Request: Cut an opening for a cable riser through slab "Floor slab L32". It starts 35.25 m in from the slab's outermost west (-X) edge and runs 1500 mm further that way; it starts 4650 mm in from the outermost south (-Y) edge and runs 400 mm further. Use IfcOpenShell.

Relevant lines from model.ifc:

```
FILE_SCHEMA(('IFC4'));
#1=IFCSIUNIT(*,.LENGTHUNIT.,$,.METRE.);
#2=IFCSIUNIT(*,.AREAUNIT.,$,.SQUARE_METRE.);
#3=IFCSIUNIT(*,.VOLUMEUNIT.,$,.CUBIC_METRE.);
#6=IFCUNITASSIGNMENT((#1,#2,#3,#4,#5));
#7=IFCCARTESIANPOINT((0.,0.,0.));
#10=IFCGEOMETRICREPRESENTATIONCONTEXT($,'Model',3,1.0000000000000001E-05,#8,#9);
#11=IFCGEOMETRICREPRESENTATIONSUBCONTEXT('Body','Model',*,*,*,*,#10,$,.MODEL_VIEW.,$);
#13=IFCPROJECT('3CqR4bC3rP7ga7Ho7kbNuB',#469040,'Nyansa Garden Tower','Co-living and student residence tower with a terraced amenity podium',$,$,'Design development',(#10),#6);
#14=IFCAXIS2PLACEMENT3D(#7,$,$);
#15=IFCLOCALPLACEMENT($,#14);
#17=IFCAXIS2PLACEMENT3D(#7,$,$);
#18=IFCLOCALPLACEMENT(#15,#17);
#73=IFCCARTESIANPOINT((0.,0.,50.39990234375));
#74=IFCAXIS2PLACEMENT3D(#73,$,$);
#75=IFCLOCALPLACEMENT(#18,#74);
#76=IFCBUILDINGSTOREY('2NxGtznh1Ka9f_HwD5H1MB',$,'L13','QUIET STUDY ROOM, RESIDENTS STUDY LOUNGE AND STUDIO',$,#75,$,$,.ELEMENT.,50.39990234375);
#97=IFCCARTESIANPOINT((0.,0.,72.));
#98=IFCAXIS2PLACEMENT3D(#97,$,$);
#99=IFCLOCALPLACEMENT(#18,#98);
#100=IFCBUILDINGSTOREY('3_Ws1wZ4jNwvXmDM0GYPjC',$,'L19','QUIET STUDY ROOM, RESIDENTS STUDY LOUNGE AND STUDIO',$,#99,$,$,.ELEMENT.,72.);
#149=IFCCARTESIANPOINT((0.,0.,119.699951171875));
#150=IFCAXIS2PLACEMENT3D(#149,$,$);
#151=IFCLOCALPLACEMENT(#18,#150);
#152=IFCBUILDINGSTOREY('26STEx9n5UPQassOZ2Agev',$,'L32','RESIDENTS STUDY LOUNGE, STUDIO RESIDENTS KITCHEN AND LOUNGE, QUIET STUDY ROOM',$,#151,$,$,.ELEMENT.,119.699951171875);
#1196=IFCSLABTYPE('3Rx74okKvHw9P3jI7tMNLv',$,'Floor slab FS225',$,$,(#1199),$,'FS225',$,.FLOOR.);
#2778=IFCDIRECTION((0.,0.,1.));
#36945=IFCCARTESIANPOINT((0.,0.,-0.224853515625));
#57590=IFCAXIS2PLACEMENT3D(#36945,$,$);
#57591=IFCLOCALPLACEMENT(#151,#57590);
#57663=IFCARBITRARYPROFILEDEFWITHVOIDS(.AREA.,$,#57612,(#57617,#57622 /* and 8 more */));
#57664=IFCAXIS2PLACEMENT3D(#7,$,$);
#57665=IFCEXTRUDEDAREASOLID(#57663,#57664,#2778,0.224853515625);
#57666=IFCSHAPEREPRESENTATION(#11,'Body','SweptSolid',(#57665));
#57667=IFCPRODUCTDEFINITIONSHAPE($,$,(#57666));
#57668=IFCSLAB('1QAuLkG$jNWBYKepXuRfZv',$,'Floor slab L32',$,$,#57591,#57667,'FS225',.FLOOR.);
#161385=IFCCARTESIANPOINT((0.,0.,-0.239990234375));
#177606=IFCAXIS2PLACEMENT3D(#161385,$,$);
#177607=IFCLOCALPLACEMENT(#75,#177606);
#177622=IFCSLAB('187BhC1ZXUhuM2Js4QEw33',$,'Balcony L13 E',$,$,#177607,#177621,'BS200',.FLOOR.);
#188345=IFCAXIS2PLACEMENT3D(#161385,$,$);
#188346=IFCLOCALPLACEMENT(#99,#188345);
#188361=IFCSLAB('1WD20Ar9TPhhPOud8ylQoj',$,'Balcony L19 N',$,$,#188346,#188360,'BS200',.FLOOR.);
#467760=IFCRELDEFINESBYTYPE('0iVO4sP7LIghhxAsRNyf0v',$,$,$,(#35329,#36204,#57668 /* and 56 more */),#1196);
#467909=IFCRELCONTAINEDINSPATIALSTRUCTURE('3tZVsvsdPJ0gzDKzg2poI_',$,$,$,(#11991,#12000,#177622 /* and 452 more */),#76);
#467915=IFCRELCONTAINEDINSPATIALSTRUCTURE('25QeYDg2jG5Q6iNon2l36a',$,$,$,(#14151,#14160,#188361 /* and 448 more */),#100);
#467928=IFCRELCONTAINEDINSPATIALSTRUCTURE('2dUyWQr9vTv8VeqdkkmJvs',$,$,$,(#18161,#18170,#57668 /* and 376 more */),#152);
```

```python
import numpy as np
import ifcopenshell
import ifcopenshell.api.feature
import ifcopenshell.api.geometry
import ifcopenshell.api.root
import ifcopenshell.geom
import ifcopenshell.util.placement
import ifcopenshell.util.representation
import ifcopenshell.util.shape
import ifcopenshell.util.unit

model = ifcopenshell.open("model.ifc")
unit_scale = ifcopenshell.util.unit.calculate_unit_scale(model)
settings = ifcopenshell.geom.settings()


def volume(element):
    """Net volume in cubic metres, openings subtracted."""
    shape = ifcopenshell.geom.create_shape(settings, element)
    return ifcopenshell.util.shape.get_volume(shape.geometry)


slab = model.by_id(57668)
before = volume(slab)

# Extent in the slab's own axes, in metres. The edges named are its -X and -Y sides.
slab_shape = ifcopenshell.geom.create_shape(settings, slab)
vertices = ifcopenshell.util.shape.get_vertices(slab_shape.geometry)
x_min, y_min, bottom = vertices.min(axis=0)
top = vertices[:, 2].max()

opening = ifcopenshell.api.root.create_entity(model, ifc_class="IfcOpeningElement", name="Cable riser opening", predefined_type="OPENING")
context = ifcopenshell.util.representation.get_context(model, "Model", "Body", "MODEL_VIEW")
width, depth = 1.5, 0.4
outline = [(0.0, 0.0), (width, 0.0), (width, depth), (0.0, depth), (0.0, 0.0)]
# Overshoot both faces by 50 mm so the cut is clean.
shape = ifcopenshell.api.geometry.add_slab_representation(
    model, context=context, depth=top - bottom + 0.1, polyline=outline
)
ifcopenshell.api.geometry.assign_representation(model, product=opening, representation=shape)

matrix = ifcopenshell.util.placement.get_local_placement(slab.ObjectPlacement)
matrix[:, 3] = matrix @ np.append(np.array([x_min + 35.25, y_min + 4.65, bottom - 0.05]) / unit_scale, 1.0)
ifcopenshell.api.geometry.edit_object_placement(model, product=opening, matrix=matrix, is_si=False)
ifcopenshell.api.feature.add_feature(model, feature=opening, element=slab)

after = volume(slab)

print(f"slab volume {before:.3f} -> {after:.3f} m3")

model.write("model_updated.ifc")
```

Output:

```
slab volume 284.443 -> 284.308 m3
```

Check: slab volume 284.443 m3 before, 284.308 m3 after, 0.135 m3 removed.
